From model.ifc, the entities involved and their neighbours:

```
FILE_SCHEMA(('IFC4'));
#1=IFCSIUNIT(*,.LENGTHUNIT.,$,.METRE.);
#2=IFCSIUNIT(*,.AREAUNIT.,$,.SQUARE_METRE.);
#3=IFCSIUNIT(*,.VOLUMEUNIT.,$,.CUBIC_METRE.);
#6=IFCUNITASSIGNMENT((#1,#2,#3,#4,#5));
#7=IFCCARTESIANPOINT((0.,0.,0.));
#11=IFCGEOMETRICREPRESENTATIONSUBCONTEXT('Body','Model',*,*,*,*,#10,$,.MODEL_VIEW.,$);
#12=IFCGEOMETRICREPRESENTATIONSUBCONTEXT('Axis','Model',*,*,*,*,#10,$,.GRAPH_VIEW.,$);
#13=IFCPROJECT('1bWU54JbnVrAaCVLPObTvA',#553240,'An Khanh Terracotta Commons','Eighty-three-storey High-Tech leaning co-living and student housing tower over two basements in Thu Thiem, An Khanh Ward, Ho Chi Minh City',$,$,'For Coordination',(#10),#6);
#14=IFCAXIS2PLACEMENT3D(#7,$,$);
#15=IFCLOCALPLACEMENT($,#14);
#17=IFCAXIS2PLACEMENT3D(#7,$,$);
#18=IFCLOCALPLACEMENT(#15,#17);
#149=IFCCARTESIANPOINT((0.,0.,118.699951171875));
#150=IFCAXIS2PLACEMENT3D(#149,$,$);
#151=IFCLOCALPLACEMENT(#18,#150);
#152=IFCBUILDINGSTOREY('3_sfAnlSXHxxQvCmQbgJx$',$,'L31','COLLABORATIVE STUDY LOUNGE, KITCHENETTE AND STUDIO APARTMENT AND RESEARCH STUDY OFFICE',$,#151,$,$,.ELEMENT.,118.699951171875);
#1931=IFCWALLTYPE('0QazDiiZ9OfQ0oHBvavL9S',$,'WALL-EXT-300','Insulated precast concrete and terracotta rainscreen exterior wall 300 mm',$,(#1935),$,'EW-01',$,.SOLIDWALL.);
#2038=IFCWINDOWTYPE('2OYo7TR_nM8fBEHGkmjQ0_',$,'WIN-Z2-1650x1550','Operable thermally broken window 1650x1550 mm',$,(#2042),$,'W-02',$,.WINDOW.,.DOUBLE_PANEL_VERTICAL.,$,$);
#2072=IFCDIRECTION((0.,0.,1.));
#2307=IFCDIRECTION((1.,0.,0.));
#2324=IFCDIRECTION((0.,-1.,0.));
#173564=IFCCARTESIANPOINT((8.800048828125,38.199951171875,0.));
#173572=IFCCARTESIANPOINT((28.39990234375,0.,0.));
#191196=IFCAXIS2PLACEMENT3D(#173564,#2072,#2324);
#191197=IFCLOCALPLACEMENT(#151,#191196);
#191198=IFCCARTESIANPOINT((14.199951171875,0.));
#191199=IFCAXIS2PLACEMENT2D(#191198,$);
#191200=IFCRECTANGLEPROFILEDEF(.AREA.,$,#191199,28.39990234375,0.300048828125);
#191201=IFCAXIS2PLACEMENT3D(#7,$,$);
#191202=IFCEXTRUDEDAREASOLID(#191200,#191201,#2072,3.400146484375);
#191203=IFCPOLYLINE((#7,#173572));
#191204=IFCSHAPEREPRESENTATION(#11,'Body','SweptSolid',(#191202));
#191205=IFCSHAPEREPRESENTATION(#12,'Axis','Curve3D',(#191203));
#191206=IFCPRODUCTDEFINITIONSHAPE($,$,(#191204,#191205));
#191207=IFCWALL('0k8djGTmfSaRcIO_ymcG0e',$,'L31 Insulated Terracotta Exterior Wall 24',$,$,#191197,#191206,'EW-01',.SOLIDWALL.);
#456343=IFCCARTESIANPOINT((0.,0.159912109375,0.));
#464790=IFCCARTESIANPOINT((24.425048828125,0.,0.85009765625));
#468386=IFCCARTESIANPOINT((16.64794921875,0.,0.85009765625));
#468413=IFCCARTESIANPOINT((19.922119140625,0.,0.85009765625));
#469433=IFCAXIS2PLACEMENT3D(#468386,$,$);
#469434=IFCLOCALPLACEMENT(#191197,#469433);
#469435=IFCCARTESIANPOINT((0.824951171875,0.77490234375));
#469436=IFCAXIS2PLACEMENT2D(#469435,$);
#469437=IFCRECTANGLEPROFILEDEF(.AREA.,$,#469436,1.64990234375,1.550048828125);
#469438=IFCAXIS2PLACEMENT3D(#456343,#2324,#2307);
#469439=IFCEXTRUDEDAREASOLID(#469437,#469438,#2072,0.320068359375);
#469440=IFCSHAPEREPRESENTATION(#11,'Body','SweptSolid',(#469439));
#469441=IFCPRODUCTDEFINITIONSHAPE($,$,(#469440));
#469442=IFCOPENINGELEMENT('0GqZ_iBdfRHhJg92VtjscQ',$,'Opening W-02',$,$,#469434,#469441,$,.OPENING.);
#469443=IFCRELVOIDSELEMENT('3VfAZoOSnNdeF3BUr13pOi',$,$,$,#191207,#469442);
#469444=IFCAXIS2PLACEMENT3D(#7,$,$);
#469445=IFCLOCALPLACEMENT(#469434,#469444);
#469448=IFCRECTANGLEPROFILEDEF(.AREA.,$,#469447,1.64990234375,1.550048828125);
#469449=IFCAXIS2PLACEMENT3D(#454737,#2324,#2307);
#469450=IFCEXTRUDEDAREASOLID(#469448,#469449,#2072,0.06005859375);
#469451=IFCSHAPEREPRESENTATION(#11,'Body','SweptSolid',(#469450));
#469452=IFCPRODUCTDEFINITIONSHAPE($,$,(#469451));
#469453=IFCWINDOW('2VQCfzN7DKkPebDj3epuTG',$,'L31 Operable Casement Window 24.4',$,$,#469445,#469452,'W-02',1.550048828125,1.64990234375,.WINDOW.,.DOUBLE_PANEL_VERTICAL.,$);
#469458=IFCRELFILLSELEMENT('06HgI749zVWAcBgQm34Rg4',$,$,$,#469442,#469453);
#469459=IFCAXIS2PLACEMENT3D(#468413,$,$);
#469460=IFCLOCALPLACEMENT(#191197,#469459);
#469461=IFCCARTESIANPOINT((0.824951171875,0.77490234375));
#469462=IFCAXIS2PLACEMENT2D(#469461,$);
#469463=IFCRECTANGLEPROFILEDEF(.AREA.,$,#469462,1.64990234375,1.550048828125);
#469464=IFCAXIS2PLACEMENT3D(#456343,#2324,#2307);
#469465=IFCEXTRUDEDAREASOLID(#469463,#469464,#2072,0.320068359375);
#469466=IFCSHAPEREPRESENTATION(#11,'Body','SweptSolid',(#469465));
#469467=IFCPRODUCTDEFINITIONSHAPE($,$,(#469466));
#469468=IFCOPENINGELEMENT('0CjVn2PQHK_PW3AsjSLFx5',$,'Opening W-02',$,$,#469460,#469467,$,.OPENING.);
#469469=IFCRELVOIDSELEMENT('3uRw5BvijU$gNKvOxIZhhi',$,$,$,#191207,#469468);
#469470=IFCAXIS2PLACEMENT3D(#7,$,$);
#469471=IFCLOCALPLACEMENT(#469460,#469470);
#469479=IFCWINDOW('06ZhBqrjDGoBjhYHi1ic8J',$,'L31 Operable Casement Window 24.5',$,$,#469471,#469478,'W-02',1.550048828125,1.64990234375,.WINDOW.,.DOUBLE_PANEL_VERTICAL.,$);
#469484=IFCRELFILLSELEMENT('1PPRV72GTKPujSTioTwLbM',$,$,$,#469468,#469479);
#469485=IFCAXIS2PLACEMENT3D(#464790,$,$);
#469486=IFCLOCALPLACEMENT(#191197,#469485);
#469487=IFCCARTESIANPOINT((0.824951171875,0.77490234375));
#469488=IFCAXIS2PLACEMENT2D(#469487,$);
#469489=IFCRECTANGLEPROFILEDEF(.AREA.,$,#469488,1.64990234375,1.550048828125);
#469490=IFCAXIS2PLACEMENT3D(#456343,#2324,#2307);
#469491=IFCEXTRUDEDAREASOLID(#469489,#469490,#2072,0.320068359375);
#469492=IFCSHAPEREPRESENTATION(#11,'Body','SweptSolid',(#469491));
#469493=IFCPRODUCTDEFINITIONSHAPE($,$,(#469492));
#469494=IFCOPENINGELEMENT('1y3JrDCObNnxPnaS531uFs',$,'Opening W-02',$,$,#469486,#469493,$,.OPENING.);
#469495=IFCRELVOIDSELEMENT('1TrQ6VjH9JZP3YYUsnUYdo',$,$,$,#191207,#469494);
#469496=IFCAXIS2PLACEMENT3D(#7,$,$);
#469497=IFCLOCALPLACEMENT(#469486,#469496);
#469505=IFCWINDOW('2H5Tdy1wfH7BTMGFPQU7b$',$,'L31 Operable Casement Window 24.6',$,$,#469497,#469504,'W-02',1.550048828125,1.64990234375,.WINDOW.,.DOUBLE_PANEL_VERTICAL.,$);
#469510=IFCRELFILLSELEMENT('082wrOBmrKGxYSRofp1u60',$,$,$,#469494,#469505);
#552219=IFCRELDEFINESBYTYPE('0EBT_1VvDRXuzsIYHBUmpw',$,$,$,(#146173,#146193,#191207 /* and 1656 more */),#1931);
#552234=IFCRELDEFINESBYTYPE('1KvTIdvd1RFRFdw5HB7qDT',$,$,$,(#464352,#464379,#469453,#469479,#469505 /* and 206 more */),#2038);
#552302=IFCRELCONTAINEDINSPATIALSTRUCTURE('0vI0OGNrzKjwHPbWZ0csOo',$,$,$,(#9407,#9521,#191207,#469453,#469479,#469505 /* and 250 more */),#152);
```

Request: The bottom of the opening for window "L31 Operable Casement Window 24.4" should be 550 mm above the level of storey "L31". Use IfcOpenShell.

```python
import numpy as np
import ifcopenshell
import ifcopenshell.api.geometry
import ifcopenshell.geom
import ifcopenshell.util.element
import ifcopenshell.util.placement
import ifcopenshell.util.shape
import ifcopenshell.util.unit

model = ifcopenshell.open("model.ifc")
unit_scale = ifcopenshell.util.unit.calculate_unit_scale(model)

window = model.by_id(469453)
opening = window.FillsVoids[0].RelatingOpeningElement
storey = ifcopenshell.util.element.get_container(window, ifc_class="IfcBuildingStorey")
level = ifcopenshell.util.placement.get_local_placement(storey.ObjectPlacement)[2, 3]

# The opening's origin need not be at the sill, so measure its lowest point.
shape = ifcopenshell.geom.create_shape(ifcopenshell.geom.settings(), opening)
bottom = ifcopenshell.util.shape.get_shape_bottom_elevation(shape, shape.geometry) / unit_scale
dz = level + 0.55 / unit_scale - bottom

shift = np.array([0.0, 0.0, dz])
# The window is placed relative to its opening, so it follows when the opening moves.
matrix = ifcopenshell.util.placement.get_local_placement(opening.ObjectPlacement)
matrix[:3, 3] += shift
ifcopenshell.api.geometry.edit_object_placement(
    model, product=opening, matrix=matrix, is_si=False, should_transform_children=True
)

print(f"moved by {dz * unit_scale:+.3f} m")

model.write("model_edited.ifc")
```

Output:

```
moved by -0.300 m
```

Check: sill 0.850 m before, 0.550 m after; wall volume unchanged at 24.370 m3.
